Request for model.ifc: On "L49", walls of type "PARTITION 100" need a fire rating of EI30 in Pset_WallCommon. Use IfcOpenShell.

First a look at what the model holds.

```python
import ifcopenshell
import ifcopenshell.util.element

model = ifcopenshell.open("model.ifc")
print(model.schema)
storey = next(s for s in model.by_type("IfcBuildingStorey") if s.Name == "L49")
walls = [e for e in ifcopenshell.util.element.get_decomposition(storey) if e.is_a("IfcWall")]
seen = {}
for e in walls:
    element_type = ifcopenshell.util.element.get_type(e)
    key = (element_type.Name if element_type != e and element_type else None, ifcopenshell.util.element.get_pset(e, "Pset_WallCommon", "FireRating"))
    seen[key] = seen.get(key, 0) + 1
for (name, value), count in sorted(seen.items(), key=str):
    print(count, "x", name, "|", value)
```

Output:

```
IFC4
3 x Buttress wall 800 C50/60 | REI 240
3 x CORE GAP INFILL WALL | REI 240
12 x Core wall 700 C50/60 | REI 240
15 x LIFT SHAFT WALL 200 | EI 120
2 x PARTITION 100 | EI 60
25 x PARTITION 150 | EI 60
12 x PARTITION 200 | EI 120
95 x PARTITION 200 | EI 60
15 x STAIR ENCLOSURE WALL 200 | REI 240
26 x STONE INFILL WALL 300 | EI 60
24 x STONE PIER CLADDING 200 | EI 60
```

```python
import ifcopenshell
import ifcopenshell.api.pset
import ifcopenshell.util.element

model = ifcopenshell.open("model.ifc")

storey = next(s for s in model.by_type("IfcBuildingStorey") if s.Name == "L49")
walls = [e for e in ifcopenshell.util.element.get_decomposition(storey) if e.is_a("IfcWall")]

count = 0
for e in walls:
    element_type = ifcopenshell.util.element.get_type(e)
    if element_type in (None, e) or element_type.Name != "PARTITION 100":
        continue
    found = ifcopenshell.util.element.get_pset(e, "Pset_WallCommon", should_inherit=False)
    if found:
        pset = model.by_id(found["id"])
        if len(ifcopenshell.util.element.get_elements_by_pset(pset)) > 1:
            pset = ifcopenshell.api.pset.unshare_pset(model, products=[e], pset=pset)[0]
    else:
        pset = ifcopenshell.api.pset.add_pset(model, product=e, name="Pset_WallCommon")
    ifcopenshell.api.pset.edit_pset(model, pset=pset, properties={"FireRating": "EI30"})
    count += 1

print(count, "walls updated")

model.write("model_updated.ifc")
```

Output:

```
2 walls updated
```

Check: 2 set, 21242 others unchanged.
